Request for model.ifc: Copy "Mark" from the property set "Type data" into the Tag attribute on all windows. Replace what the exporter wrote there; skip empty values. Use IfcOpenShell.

First a look at what the model holds.

```python
import ifcopenshell
import ifcopenshell.util.element

model = ifcopenshell.open("model.ifc")
print(model.schema)
windows = model.by_type("IfcWindow")
print(len(windows), "windows")
for e in windows[:8]:
    source = ifcopenshell.util.element.get_pset(e, "Type data", "Mark")
    target = e.Tag
    print(e.id(), repr(source), repr(target), sep=" | ")
```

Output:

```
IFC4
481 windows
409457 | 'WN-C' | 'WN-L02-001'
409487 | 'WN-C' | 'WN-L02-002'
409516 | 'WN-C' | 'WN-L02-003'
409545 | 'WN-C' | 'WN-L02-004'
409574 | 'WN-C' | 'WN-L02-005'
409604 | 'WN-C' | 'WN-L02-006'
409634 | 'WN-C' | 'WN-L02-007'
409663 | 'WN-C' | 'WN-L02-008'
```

```python
import ifcopenshell
import ifcopenshell.util.element

model = ifcopenshell.open("model.ifc")

count = 0
for e in model.by_type("IfcWindow"):
    value = ifcopenshell.util.element.get_pset(e, "Type data", "Mark")
    current = e.Tag
    if not value or not value.strip() or current == value:
        continue
    e.Tag = value
    count += 1

print(count, "windows updated")

model.write("model_edited.ifc")
```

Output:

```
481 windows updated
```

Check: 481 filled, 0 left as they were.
